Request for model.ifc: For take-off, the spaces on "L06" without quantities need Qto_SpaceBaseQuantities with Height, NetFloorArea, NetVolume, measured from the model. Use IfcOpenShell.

First a look at what the model holds.

```python
import ifcopenshell
import ifcopenshell.util.element
import ifcopenshell.util.unit

model = ifcopenshell.open("model.ifc")
print(model.schema)
for unit_type in ("LENGTHUNIT", "AREAUNIT", "VOLUMEUNIT"):
    print(unit_type, ifcopenshell.util.unit.calculate_unit_scale(model, unit_type))
storey = next(s for s in model.by_type("IfcBuildingStorey") if s.Name == "L06")
spaces = [e for e in ifcopenshell.util.element.get_decomposition(storey) if e.is_a("IfcSpace")]
for e in sorted(spaces, key=lambda e: e.id()):
    print(e.id(), e.is_a(), e.Name, list(ifcopenshell.util.element.get_psets(e, qtos_only=True)), sep=" | ")
```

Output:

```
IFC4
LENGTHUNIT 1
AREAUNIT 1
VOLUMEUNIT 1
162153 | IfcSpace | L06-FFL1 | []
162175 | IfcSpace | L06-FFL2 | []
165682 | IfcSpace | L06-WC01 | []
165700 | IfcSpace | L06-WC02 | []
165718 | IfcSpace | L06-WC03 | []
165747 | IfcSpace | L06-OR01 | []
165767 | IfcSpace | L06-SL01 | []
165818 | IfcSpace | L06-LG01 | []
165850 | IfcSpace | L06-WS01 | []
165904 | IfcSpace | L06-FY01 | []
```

```python
import ifcopenshell
import ifcopenshell.api.pset
import ifcopenshell.geom
import ifcopenshell.util.element
import ifcopenshell.util.shape
import ifcopenshell.util.unit

model = ifcopenshell.open("model.ifc")
unit_scale = ifcopenshell.util.unit.calculate_unit_scale(model)
area_scale = ifcopenshell.util.unit.calculate_unit_scale(model, "AREAUNIT")
volume_scale = ifcopenshell.util.unit.calculate_unit_scale(model, "VOLUMEUNIT")
settings = ifcopenshell.geom.settings()

storey = next(s for s in model.by_type("IfcBuildingStorey") if s.Name == "L06")
spaces = [e for e in ifcopenshell.util.element.get_decomposition(storey) if e.is_a("IfcSpace")]

for e in sorted(spaces, key=lambda e: e.id()):
    if ifcopenshell.util.element.get_psets(e, qtos_only=True, should_inherit=False):
        continue
    # Geometry comes back in metres, in the element's own axes.
    shape = ifcopenshell.geom.create_shape(settings, e)
    values = {
        "Height": ifcopenshell.util.shape.get_z(shape.geometry) / unit_scale,
        "NetFloorArea": ifcopenshell.util.shape.get_footprint_area(shape.geometry) / area_scale,
        "NetVolume": ifcopenshell.util.shape.get_volume(shape.geometry) / volume_scale,
    }
    qto = ifcopenshell.api.pset.add_qto(model, product=e, name="Qto_SpaceBaseQuantities")
    ifcopenshell.api.pset.edit_qto(model, qto=qto, properties=values)
    print(e.id(), {k: round(v, 3) for k, v in values.items()})

model.write("model_v2.ifc")
```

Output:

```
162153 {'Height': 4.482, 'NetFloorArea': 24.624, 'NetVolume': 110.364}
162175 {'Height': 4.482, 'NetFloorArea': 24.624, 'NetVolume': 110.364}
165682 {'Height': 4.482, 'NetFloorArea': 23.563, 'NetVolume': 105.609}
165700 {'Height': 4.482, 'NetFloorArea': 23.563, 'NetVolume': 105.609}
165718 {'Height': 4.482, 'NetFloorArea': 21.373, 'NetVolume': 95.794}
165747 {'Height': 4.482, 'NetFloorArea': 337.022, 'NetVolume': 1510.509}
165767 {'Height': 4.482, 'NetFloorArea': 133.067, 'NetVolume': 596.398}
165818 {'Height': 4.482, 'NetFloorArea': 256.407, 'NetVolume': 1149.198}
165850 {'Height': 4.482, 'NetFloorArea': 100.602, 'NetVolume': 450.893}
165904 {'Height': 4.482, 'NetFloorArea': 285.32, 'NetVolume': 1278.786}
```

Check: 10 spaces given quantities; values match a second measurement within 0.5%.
